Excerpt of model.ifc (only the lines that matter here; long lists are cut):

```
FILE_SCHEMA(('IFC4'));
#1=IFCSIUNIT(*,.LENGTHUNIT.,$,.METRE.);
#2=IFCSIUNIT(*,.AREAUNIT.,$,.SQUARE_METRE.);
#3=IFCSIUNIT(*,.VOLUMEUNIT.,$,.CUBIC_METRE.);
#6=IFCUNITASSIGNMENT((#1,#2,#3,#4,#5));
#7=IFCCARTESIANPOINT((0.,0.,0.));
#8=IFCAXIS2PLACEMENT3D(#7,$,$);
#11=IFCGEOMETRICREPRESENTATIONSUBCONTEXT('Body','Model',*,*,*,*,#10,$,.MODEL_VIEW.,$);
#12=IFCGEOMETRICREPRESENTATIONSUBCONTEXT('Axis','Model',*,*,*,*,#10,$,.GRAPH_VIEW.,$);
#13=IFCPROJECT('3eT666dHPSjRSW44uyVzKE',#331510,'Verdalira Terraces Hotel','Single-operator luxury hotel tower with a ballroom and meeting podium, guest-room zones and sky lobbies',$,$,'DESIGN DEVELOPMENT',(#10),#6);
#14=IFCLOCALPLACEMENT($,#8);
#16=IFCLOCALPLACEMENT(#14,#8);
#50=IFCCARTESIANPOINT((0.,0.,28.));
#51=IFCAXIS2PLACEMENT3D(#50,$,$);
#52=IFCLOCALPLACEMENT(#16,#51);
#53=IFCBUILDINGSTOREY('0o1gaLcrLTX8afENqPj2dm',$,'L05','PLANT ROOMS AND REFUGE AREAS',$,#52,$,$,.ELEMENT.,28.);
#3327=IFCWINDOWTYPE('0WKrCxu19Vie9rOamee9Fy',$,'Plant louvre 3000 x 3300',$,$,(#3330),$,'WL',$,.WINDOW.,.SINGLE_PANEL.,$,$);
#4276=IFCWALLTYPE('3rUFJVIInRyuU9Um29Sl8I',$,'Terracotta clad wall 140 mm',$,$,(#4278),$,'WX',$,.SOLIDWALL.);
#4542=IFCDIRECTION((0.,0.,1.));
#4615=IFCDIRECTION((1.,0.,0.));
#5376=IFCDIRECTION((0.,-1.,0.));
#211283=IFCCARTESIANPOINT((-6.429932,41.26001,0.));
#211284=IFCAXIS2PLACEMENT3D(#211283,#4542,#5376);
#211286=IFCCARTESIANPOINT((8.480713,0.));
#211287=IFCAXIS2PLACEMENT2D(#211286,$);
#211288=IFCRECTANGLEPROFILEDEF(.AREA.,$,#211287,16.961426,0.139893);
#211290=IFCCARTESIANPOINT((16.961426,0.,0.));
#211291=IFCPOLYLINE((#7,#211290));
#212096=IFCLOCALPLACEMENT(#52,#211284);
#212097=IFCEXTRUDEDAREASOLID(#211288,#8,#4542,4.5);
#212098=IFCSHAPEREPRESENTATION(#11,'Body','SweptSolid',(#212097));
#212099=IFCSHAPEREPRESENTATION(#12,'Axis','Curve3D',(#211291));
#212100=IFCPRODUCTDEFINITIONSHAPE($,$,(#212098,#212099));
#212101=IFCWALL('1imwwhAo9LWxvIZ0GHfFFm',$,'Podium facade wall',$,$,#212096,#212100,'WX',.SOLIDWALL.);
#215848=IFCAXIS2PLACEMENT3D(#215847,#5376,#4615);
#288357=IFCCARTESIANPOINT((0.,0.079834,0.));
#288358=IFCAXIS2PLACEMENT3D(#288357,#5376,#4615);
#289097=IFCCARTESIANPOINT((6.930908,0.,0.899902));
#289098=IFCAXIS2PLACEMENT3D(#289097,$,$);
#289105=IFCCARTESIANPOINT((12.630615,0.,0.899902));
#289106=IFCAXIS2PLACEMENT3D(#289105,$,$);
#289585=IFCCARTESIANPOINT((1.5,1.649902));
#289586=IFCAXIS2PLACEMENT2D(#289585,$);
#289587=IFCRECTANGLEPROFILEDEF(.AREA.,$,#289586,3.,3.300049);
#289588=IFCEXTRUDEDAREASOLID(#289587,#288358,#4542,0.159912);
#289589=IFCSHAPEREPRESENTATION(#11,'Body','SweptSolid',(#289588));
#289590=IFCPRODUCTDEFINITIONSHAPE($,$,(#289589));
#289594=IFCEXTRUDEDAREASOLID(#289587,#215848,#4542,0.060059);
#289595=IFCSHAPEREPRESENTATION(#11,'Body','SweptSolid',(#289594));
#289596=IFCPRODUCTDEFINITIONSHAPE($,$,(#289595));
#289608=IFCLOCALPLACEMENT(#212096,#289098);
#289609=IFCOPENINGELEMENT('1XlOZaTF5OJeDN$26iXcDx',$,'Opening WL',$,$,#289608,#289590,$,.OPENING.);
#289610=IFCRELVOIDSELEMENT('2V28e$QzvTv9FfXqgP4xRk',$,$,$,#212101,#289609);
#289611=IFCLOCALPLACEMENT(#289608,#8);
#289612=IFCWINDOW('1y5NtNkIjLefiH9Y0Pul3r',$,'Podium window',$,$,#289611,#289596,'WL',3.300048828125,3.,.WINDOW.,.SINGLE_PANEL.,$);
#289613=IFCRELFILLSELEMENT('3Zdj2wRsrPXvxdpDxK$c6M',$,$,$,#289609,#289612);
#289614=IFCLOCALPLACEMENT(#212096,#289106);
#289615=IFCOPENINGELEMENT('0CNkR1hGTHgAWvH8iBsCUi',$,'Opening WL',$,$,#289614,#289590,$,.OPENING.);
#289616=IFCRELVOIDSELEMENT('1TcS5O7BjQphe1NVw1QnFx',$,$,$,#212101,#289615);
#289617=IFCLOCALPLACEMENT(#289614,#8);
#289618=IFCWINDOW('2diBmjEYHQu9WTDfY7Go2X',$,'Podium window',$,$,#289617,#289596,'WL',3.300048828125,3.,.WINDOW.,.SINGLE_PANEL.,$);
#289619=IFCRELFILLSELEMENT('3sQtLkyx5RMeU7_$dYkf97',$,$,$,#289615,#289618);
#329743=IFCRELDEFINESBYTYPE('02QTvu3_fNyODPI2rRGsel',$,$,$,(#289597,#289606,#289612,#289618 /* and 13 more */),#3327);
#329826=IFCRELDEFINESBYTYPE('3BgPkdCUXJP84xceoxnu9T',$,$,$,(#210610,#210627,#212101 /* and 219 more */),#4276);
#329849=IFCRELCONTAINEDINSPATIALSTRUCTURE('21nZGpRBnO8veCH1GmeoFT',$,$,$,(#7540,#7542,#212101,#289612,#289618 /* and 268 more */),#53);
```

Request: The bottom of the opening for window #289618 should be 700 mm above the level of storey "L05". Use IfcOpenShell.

```python
import numpy as np
import ifcopenshell
import ifcopenshell.api.geometry
import ifcopenshell.geom
import ifcopenshell.util.element
import ifcopenshell.util.placement
import ifcopenshell.util.shape
import ifcopenshell.util.unit

model = ifcopenshell.open("model.ifc")
unit_scale = ifcopenshell.util.unit.calculate_unit_scale(model)

window = model.by_guid("2diBmjEYHQu9WTDfY7Go2X")
opening = window.FillsVoids[0].RelatingOpeningElement
storey = ifcopenshell.util.element.get_container(window, ifc_class="IfcBuildingStorey")
level = ifcopenshell.util.placement.get_local_placement(storey.ObjectPlacement)[2, 3]

# The opening's origin need not be at the sill, so measure its lowest point.
shape = ifcopenshell.geom.create_shape(ifcopenshell.geom.settings(), opening)
bottom = ifcopenshell.util.shape.get_shape_bottom_elevation(shape, shape.geometry) / unit_scale
dz = level + 0.7 / unit_scale - bottom

shift = np.array([0.0, 0.0, dz])
# The window is placed relative to its opening, so it follows when the opening moves.
matrix = ifcopenshell.util.placement.get_local_placement(opening.ObjectPlacement)
matrix[:3, 3] += shift
ifcopenshell.api.geometry.edit_object_placement(
    model, product=opening, matrix=matrix, is_si=False, should_transform_children=True
)

print(f"moved by {dz * unit_scale:+.3f} m")

model.write("model_edited.ifc")
```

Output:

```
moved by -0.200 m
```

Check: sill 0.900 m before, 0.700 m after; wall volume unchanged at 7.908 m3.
